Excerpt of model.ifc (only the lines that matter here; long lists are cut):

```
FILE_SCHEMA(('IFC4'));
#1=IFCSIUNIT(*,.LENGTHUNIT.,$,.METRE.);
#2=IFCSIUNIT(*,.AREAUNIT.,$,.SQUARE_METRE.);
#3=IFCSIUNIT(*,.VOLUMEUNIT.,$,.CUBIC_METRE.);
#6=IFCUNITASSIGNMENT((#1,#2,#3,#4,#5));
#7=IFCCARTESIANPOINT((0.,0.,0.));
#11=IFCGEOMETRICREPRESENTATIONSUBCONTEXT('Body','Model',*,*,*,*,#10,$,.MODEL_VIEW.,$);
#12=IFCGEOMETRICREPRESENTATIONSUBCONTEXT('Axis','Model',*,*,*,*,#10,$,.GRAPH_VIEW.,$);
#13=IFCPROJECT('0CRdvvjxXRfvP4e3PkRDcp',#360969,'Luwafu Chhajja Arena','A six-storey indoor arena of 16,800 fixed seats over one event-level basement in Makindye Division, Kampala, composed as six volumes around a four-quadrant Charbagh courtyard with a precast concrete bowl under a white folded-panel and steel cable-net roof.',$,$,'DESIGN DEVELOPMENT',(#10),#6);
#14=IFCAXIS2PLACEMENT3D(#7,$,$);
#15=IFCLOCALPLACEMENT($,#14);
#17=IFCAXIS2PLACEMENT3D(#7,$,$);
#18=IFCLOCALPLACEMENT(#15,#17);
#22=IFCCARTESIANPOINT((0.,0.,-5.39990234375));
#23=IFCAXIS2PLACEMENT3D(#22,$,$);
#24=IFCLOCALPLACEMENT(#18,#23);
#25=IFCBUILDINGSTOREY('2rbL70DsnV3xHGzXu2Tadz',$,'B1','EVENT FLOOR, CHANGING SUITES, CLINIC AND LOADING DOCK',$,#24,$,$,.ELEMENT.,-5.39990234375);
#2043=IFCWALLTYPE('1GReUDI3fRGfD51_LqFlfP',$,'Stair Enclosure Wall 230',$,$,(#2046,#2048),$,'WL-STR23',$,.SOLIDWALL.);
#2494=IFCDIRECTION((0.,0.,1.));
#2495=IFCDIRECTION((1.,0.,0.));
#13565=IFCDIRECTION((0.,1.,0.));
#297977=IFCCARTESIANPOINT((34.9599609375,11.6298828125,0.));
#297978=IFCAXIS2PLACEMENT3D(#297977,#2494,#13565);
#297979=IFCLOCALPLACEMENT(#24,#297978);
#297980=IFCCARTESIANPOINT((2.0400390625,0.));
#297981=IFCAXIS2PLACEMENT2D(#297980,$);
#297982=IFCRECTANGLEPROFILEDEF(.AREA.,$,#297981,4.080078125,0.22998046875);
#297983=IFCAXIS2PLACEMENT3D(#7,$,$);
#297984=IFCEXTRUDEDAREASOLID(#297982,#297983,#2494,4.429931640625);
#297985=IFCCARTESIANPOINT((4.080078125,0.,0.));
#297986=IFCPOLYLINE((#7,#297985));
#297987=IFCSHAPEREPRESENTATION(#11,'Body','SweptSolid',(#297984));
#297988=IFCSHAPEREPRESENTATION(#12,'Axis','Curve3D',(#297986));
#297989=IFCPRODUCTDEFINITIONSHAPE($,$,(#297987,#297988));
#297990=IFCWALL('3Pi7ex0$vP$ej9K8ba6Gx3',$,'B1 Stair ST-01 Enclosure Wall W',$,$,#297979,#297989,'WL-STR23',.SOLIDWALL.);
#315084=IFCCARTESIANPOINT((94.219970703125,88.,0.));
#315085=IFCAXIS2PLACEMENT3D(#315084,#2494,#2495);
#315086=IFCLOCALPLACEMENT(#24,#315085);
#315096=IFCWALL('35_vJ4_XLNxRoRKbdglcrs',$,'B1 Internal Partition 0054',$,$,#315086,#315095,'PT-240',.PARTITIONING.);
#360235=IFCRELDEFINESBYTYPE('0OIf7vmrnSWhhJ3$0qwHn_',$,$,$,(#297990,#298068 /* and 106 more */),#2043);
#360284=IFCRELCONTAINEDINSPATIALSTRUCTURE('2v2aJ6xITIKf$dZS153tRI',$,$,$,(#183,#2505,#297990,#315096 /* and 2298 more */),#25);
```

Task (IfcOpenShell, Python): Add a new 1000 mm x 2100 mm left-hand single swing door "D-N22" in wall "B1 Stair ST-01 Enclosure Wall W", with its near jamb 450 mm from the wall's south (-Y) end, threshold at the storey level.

```python
import numpy as np
import ifcopenshell
import ifcopenshell.api.feature
import ifcopenshell.api.geometry
import ifcopenshell.api.root
import ifcopenshell.api.spatial
import ifcopenshell.geom
import ifcopenshell.util.element
import ifcopenshell.util.placement
import ifcopenshell.util.representation
import ifcopenshell.util.shape
import ifcopenshell.util.unit

model = ifcopenshell.open("model.ifc")
unit_scale = ifcopenshell.util.unit.calculate_unit_scale(model)
settings = ifcopenshell.geom.settings()


def volume(element):
    """Net volume in cubic metres, openings subtracted."""
    shape = ifcopenshell.geom.create_shape(settings, element)
    return ifcopenshell.util.shape.get_volume(shape.geometry)


wall = model.by_guid("3Pi7ex0$vP$ej9K8ba6Gx3")
storey = ifcopenshell.util.element.get_container(wall, ifc_class="IfcBuildingStorey")
context = ifcopenshell.util.representation.get_context(model, "Model", "Body", "MODEL_VIEW")
before = volume(wall)

width, height, from_end, sill = 1, 2.1, 0.45, 0.0  # metres

# The wall runs along its own X axis, and the end named is its -X end.
wall_shape = ifcopenshell.geom.create_shape(settings, wall)
x, y, z = ifcopenshell.util.shape.get_vertices(wall_shape.geometry).T
start = x.min() + from_end
face, thickness = float(y.min()), float(y.max() - y.min())
wall_matrix = ifcopenshell.util.placement.get_local_placement(wall.ObjectPlacement)
level = ifcopenshell.util.placement.get_local_placement(storey.ObjectPlacement)[2, 3]


def in_wall(x, y):
    """Placement at x, y metres in the wall's axes, at sill height."""
    matrix = wall_matrix.copy()
    matrix[:, 3] = wall_matrix @ np.array([x / unit_scale, y / unit_scale, 0.0, 1.0])
    matrix[2, 3] = level + sill / unit_scale
    return matrix


# Opening: a box that overshoots both wall faces by 50 mm.
opening = ifcopenshell.api.root.create_entity(model, ifc_class="IfcOpeningElement", predefined_type="OPENING")
box = ifcopenshell.api.geometry.add_wall_representation(
    model, context=context, length=width, height=height, thickness=thickness + 0.1
)
ifcopenshell.api.geometry.assign_representation(model, product=opening, representation=box)
ifcopenshell.api.geometry.edit_object_placement(model, product=opening, matrix=in_wall(start, face - 0.05), is_si=False)
ifcopenshell.api.feature.add_feature(model, feature=opening, element=wall)

door = ifcopenshell.api.root.create_entity(model, ifc_class="IfcDoor", name="D-N22", predefined_type="DOOR")
door.OverallWidth, door.OverallHeight = width / unit_scale, height / unit_scale
door.OperationType = "SINGLE_SWING_LEFT"
body = ifcopenshell.api.geometry.add_door_representation(
    model,
    context=context,
    overall_width=door.OverallWidth,
    overall_height=door.OverallHeight,
    operation_type="SINGLE_SWING_LEFT",
    lining_properties={"LiningDepth": thickness / unit_scale, "ThresholdDepth": thickness / unit_scale},
)
ifcopenshell.api.geometry.assign_representation(model, product=door, representation=body)
ifcopenshell.api.spatial.assign_container(model, products=[door], relating_structure=storey)
ifcopenshell.api.feature.add_filling(model, opening=opening, element=door)

# The lining spans the wall, so the door starts at the wall face.
ifcopenshell.api.geometry.edit_object_placement(model, product=door, matrix=in_wall(start, face), is_si=False)

after = volume(wall)

print(f"wall volume {before:.3f} -> {after:.3f} m3")

model.write("model-out.ifc")
```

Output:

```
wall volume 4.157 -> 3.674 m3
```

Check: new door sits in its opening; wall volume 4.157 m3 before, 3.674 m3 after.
